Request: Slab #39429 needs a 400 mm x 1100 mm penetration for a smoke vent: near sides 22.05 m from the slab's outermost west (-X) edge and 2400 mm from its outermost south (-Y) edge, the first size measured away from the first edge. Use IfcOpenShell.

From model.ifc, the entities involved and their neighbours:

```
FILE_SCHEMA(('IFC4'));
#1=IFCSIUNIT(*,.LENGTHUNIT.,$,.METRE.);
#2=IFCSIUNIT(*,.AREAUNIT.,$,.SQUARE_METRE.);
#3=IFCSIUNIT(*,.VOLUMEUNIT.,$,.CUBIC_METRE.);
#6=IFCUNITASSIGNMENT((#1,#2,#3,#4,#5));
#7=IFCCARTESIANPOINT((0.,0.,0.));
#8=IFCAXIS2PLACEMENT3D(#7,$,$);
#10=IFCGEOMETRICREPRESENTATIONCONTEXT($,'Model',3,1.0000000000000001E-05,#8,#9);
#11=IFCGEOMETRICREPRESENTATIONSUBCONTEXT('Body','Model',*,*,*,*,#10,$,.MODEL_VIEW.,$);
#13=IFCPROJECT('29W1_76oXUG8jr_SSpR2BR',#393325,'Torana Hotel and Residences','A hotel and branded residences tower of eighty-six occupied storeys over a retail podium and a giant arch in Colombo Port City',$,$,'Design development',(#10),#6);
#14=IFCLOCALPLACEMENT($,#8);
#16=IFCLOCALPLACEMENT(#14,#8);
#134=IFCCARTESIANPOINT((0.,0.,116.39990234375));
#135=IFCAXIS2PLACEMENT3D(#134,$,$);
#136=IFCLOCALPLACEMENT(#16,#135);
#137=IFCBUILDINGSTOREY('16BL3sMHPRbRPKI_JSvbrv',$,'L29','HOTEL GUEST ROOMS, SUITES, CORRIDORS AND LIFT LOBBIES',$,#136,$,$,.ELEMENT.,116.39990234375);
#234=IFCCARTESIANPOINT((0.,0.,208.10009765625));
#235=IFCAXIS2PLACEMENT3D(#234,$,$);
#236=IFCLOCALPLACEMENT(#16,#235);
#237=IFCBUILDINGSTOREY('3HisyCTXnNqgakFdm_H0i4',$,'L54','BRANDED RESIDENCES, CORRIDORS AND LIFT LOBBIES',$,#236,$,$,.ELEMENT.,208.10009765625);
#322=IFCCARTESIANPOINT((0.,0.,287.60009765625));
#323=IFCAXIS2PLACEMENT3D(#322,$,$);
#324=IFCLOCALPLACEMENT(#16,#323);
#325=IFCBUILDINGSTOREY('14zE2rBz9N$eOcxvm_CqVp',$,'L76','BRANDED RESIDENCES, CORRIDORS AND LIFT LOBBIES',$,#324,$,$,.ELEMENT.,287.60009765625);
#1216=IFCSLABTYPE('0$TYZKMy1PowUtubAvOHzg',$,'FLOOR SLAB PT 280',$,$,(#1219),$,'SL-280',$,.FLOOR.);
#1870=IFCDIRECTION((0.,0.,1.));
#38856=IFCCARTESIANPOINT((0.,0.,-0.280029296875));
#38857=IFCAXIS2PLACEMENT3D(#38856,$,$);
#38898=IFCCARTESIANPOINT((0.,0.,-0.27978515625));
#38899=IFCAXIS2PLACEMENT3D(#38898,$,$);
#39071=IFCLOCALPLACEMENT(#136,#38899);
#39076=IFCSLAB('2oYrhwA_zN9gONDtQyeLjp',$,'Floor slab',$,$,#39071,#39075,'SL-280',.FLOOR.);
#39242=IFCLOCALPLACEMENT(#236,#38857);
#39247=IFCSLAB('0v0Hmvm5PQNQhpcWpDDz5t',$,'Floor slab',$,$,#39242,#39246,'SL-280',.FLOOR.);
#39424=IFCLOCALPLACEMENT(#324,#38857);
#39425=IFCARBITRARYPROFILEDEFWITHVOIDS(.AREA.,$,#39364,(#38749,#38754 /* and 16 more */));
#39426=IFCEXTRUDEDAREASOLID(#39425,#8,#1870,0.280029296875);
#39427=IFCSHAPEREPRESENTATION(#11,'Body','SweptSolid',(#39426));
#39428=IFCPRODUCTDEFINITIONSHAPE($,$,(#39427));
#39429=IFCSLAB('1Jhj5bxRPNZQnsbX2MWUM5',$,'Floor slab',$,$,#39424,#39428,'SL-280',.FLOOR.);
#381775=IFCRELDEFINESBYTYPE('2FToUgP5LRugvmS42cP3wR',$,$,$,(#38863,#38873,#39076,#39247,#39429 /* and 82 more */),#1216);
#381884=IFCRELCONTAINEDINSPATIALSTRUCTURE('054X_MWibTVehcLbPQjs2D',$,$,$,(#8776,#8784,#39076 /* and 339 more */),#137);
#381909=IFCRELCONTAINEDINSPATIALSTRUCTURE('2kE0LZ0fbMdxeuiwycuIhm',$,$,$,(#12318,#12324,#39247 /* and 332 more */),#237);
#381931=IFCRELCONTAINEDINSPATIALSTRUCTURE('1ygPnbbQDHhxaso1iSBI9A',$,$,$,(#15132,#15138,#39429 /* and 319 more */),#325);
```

```python
import numpy as np
import ifcopenshell
import ifcopenshell.api.feature
import ifcopenshell.api.geometry
import ifcopenshell.api.root
import ifcopenshell.geom
import ifcopenshell.util.placement
import ifcopenshell.util.representation
import ifcopenshell.util.shape
import ifcopenshell.util.unit

model = ifcopenshell.open("model.ifc")
unit_scale = ifcopenshell.util.unit.calculate_unit_scale(model)
settings = ifcopenshell.geom.settings()


def volume(element):
    """Net volume in cubic metres, openings subtracted."""
    shape = ifcopenshell.geom.create_shape(settings, element)
    return ifcopenshell.util.shape.get_volume(shape.geometry)


slab = model.by_id(39429)
before = volume(slab)

# Extent in the slab's own axes, in metres. The edges named are its -X and -Y sides.
slab_shape = ifcopenshell.geom.create_shape(settings, slab)
vertices = ifcopenshell.util.shape.get_vertices(slab_shape.geometry)
x_min, y_min, bottom = vertices.min(axis=0)
top = vertices[:, 2].max()

opening = ifcopenshell.api.root.create_entity(model, ifc_class="IfcOpeningElement", name="Smoke vent opening", predefined_type="OPENING")
context = ifcopenshell.util.representation.get_context(model, "Model", "Body", "MODEL_VIEW")
width, depth = 0.4, 1.1
outline = [(0.0, 0.0), (width, 0.0), (width, depth), (0.0, depth), (0.0, 0.0)]
# Overshoot both faces by 50 mm so the cut is clean.
shape = ifcopenshell.api.geometry.add_slab_representation(
    model, context=context, depth=top - bottom + 0.1, polyline=outline
)
ifcopenshell.api.geometry.assign_representation(model, product=opening, representation=shape)

matrix = ifcopenshell.util.placement.get_local_placement(slab.ObjectPlacement)
matrix[:, 3] = matrix @ np.append(np.array([x_min + 22.05, y_min + 2.4, bottom - 0.05]) / unit_scale, 1.0)
ifcopenshell.api.geometry.edit_object_placement(model, product=opening, matrix=matrix, is_si=False)
ifcopenshell.api.feature.add_feature(model, feature=opening, element=slab)

after = volume(slab)

print(f"slab volume {before:.3f} -> {after:.3f} m3")

model.write("model-out.ifc")
```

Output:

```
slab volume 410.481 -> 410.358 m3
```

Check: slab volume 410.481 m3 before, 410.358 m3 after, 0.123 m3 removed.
